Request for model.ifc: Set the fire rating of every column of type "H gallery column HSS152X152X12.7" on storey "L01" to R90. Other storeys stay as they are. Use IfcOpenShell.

First a look at what the model holds.

```python
import ifcopenshell
import ifcopenshell.util.element

model = ifcopenshell.open("model.ifc")
print(model.schema)
storey = next(s for s in model.by_type("IfcBuildingStorey") if s.Name == "L01")
columns = [e for e in ifcopenshell.util.element.get_decomposition(storey) if e.is_a("IfcColumn")]
seen = {}
for e in columns:
    element_type = ifcopenshell.util.element.get_type(e)
    key = (element_type.Name if element_type != e and element_type else None, ifcopenshell.util.element.get_pset(e, "Pset_ColumnCommon", "FireRating"))
    seen[key] = seen.get(key, 0) + 1
for (name, value), count in sorted(seen.items(), key=str):
    print(count, "x", name, "|", value)
```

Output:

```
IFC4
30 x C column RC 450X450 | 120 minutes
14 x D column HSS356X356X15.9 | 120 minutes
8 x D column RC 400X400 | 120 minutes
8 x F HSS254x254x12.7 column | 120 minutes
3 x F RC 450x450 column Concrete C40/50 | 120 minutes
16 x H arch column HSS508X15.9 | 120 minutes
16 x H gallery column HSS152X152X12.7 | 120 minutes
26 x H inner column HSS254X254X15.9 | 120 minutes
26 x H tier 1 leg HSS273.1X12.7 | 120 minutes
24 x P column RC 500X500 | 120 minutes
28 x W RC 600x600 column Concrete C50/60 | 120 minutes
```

```python
import ifcopenshell
import ifcopenshell.api.pset
import ifcopenshell.util.element

model = ifcopenshell.open("model.ifc")

storey = next(s for s in model.by_type("IfcBuildingStorey") if s.Name == "L01")
columns = [e for e in ifcopenshell.util.element.get_decomposition(storey) if e.is_a("IfcColumn")]

count = 0
for e in columns:
    element_type = ifcopenshell.util.element.get_type(e)
    if element_type in (None, e) or element_type.Name != "H gallery column HSS152X152X12.7":
        continue
    # add_pset returns the element's existing set when there is one.
    pset = ifcopenshell.api.pset.add_pset(model, product=e, name="Pset_ColumnCommon")
    ifcopenshell.api.pset.edit_pset(model, pset=pset, properties={"FireRating": "R90"})
    count += 1

print(count, "columns updated")

model.write("model_rev.ifc")
```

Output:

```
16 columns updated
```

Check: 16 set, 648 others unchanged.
